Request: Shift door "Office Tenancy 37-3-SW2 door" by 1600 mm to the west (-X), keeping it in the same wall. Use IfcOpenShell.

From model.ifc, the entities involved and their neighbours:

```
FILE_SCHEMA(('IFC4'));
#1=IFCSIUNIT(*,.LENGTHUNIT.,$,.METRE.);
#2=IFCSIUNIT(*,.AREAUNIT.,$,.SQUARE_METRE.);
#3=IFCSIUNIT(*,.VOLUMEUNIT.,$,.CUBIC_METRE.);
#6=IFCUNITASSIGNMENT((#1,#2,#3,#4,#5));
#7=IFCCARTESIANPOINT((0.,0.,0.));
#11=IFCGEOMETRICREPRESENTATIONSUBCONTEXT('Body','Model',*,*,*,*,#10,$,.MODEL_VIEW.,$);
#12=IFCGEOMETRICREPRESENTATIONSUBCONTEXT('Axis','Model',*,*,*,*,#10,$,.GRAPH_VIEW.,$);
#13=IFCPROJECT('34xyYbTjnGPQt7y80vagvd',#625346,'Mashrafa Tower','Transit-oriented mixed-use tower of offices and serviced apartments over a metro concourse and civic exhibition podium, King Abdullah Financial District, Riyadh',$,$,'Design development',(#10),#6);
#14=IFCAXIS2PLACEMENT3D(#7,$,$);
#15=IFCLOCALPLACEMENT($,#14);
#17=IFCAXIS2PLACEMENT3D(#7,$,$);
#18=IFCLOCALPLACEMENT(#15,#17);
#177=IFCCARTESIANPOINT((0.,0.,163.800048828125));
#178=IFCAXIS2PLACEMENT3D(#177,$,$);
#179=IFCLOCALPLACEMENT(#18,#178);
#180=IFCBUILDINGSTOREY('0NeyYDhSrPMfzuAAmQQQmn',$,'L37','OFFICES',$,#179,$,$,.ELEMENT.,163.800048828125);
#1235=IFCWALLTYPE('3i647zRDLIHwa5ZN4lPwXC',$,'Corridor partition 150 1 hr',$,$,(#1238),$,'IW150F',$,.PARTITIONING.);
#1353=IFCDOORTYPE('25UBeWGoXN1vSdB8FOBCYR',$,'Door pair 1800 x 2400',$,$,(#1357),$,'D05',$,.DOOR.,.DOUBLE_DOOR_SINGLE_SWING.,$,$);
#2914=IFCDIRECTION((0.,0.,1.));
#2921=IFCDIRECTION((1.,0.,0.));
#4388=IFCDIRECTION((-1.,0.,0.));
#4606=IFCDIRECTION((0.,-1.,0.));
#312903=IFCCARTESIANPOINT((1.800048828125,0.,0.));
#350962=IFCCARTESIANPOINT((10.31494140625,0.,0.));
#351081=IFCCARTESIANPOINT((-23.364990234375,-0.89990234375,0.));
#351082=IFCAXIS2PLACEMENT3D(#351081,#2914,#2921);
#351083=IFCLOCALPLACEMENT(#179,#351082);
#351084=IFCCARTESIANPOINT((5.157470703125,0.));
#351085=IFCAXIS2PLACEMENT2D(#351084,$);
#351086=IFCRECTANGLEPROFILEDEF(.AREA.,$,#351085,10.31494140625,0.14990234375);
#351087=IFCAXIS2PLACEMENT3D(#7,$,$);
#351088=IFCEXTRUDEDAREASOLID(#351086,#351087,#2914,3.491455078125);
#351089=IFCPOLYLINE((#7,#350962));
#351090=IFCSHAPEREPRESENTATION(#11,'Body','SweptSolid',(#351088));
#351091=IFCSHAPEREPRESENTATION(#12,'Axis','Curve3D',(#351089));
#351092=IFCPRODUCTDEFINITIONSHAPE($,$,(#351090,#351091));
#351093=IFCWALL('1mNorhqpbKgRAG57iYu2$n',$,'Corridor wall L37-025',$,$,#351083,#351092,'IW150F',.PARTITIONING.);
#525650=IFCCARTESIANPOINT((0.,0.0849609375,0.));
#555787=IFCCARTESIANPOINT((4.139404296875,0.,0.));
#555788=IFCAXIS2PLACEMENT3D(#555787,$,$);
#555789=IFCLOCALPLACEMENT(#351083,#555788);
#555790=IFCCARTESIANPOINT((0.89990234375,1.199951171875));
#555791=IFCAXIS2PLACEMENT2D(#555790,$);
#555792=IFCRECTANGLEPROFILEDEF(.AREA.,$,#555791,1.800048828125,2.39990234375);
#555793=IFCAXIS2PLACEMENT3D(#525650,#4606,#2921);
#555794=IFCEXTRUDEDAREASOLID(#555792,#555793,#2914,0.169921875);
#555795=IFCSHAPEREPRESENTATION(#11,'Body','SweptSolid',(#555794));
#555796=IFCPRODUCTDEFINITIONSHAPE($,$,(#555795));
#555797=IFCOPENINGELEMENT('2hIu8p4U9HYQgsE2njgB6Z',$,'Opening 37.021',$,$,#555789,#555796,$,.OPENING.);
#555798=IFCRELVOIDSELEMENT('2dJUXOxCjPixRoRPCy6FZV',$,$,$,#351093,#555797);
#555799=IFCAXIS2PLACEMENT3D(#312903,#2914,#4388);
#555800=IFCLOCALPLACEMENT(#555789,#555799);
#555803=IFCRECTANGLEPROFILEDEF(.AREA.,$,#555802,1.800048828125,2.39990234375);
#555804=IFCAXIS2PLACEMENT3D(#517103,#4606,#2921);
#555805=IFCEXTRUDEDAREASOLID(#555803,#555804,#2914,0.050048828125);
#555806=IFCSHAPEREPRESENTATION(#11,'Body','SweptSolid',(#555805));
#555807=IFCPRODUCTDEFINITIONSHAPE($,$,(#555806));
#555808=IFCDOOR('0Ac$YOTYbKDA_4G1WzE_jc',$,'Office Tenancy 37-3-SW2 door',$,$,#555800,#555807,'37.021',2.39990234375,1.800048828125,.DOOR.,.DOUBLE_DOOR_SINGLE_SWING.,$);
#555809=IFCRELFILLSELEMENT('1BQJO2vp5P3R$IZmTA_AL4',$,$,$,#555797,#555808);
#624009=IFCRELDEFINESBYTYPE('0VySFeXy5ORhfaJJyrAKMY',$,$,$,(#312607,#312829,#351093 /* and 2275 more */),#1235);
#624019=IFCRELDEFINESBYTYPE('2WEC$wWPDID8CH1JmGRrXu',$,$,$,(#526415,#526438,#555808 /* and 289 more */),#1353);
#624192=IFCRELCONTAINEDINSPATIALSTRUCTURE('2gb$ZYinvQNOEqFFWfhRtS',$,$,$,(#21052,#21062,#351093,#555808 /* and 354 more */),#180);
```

```python
import ifcopenshell
import ifcopenshell.api.geometry
import ifcopenshell.util.placement

model = ifcopenshell.open("model.ifc")

door = model.by_guid("0Ac$YOTYbKDA_4G1WzE_jc")
opening = door.FillsVoids[0].RelatingOpeningElement
wall = opening.VoidsElements[0].RelatingBuildingElement

wall_matrix = ifcopenshell.util.placement.get_local_placement(wall.ObjectPlacement)
shift = wall_matrix[:3, 0] * -1.6
before = ifcopenshell.util.placement.get_local_placement(door.ObjectPlacement)[:3, 3].copy()

# The door is placed relative to its opening, so it follows when the opening moves.
matrix = ifcopenshell.util.placement.get_local_placement(opening.ObjectPlacement)
matrix[:3, 3] += shift
ifcopenshell.api.geometry.edit_object_placement(
    model, product=opening, matrix=matrix, is_si=False, should_transform_children=True
)

after = ifcopenshell.util.placement.get_local_placement(door.ObjectPlacement)[:3, 3]
print("door moved by", (after - before).round(3) + 0.0)

model.write("model_rev.ifc")
```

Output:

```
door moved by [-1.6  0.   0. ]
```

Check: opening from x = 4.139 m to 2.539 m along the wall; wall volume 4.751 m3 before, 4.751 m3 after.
